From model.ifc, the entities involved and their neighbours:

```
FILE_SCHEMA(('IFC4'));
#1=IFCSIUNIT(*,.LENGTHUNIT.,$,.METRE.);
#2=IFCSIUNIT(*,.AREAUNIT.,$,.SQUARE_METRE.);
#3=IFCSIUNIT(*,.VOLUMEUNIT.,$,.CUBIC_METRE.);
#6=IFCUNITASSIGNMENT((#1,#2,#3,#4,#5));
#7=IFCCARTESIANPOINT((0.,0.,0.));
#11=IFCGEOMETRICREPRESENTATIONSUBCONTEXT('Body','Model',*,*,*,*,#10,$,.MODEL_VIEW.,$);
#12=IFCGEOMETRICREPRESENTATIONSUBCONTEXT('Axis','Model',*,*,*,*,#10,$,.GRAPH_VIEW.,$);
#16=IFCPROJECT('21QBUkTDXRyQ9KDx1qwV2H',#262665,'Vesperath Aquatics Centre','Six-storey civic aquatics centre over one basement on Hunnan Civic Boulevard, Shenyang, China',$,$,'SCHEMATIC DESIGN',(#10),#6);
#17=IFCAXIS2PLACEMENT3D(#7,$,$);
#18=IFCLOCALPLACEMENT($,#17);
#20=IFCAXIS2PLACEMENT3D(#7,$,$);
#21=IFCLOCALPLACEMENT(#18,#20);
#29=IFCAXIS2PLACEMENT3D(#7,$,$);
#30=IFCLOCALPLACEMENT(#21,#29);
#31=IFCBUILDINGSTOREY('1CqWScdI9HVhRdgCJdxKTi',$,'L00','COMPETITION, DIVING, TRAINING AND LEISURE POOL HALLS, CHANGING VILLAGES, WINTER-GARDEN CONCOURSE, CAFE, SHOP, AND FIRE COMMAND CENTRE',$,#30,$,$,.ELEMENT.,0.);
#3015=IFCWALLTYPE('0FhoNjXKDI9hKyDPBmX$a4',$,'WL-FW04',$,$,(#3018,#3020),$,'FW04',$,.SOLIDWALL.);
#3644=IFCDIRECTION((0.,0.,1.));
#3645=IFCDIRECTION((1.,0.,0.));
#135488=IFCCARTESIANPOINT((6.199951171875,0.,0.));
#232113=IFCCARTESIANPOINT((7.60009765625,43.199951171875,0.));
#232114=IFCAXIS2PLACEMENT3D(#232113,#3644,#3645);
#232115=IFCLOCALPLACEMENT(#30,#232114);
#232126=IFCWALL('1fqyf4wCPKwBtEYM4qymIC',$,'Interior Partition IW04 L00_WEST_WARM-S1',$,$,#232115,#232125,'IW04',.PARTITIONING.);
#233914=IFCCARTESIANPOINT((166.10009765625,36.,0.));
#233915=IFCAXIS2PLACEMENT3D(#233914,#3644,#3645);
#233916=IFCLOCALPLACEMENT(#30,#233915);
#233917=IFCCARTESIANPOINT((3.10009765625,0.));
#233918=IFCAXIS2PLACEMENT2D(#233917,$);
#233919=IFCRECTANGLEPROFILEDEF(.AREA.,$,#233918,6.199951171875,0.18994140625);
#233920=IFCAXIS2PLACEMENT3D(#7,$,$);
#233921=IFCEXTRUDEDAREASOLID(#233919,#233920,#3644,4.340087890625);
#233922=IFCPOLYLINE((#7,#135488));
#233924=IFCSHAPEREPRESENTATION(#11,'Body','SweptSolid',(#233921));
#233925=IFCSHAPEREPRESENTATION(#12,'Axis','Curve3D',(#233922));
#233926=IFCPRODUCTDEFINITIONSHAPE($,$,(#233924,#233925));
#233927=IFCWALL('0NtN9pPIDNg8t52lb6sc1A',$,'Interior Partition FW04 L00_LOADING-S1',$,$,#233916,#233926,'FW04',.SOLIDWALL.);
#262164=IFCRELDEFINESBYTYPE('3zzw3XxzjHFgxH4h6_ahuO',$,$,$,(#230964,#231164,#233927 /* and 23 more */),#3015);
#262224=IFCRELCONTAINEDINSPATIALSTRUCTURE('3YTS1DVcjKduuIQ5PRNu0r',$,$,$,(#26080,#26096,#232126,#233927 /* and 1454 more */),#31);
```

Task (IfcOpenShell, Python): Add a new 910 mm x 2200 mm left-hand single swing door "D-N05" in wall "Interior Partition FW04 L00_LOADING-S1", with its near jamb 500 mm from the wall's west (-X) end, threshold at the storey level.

```python
import numpy as np
import ifcopenshell
import ifcopenshell.api.feature
import ifcopenshell.api.geometry
import ifcopenshell.api.root
import ifcopenshell.api.spatial
import ifcopenshell.geom
import ifcopenshell.util.element
import ifcopenshell.util.placement
import ifcopenshell.util.representation
import ifcopenshell.util.shape
import ifcopenshell.util.unit

model = ifcopenshell.open("model.ifc")
unit_scale = ifcopenshell.util.unit.calculate_unit_scale(model)
settings = ifcopenshell.geom.settings()


def volume(element):
    """Net volume in cubic metres, openings subtracted."""
    shape = ifcopenshell.geom.create_shape(settings, element)
    return ifcopenshell.util.shape.get_volume(shape.geometry)


wall = model.by_id(233927)
storey = ifcopenshell.util.element.get_container(wall, ifc_class="IfcBuildingStorey")
context = ifcopenshell.util.representation.get_context(model, "Model", "Body", "MODEL_VIEW")
before = volume(wall)

width, height, from_end, sill = 0.91, 2.2, 0.5, 0.0  # metres

# The wall runs along its own X axis, and the end named is its -X end.
wall_shape = ifcopenshell.geom.create_shape(settings, wall)
x, y, z = ifcopenshell.util.shape.get_vertices(wall_shape.geometry).T
start = x.min() + from_end
face, thickness = float(y.min()), float(y.max() - y.min())
wall_matrix = ifcopenshell.util.placement.get_local_placement(wall.ObjectPlacement)
level = ifcopenshell.util.placement.get_local_placement(storey.ObjectPlacement)[2, 3]


def in_wall(x, y):
    """Placement at x, y metres in the wall's axes, at sill height."""
    matrix = wall_matrix.copy()
    matrix[:, 3] = wall_matrix @ np.array([x / unit_scale, y / unit_scale, 0.0, 1.0])
    matrix[2, 3] = level + sill / unit_scale
    return matrix


# Opening: a box that overshoots both wall faces by 50 mm.
opening = ifcopenshell.api.root.create_entity(model, ifc_class="IfcOpeningElement", predefined_type="OPENING")
box = ifcopenshell.api.geometry.add_wall_representation(
    model, context=context, length=width, height=height, thickness=thickness + 0.1
)
ifcopenshell.api.geometry.assign_representation(model, product=opening, representation=box)
ifcopenshell.api.geometry.edit_object_placement(model, product=opening, matrix=in_wall(start, face - 0.05), is_si=False)
ifcopenshell.api.feature.add_feature(model, feature=opening, element=wall)

door = ifcopenshell.api.root.create_entity(model, ifc_class="IfcDoor", name="D-N05", predefined_type="DOOR")
door.OverallWidth, door.OverallHeight = width / unit_scale, height / unit_scale
door.OperationType = "SINGLE_SWING_LEFT"
body = ifcopenshell.api.geometry.add_door_representation(
    model,
    context=context,
    overall_width=door.OverallWidth,
    overall_height=door.OverallHeight,
    operation_type="SINGLE_SWING_LEFT",
    lining_properties={"LiningDepth": thickness / unit_scale, "ThresholdDepth": thickness / unit_scale},
)
ifcopenshell.api.geometry.assign_representation(model, product=door, representation=body)
ifcopenshell.api.spatial.assign_container(model, products=[door], relating_structure=storey)
ifcopenshell.api.feature.add_filling(model, opening=opening, element=door)

# The lining spans the wall, so the door starts at the wall face.
ifcopenshell.api.geometry.edit_object_placement(model, product=door, matrix=in_wall(start, face), is_si=False)

after = volume(wall)

print(f"wall volume {before:.3f} -> {after:.3f} m3")

model.write("model_edited.ifc")
```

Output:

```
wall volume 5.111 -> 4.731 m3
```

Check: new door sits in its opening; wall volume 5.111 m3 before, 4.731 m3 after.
